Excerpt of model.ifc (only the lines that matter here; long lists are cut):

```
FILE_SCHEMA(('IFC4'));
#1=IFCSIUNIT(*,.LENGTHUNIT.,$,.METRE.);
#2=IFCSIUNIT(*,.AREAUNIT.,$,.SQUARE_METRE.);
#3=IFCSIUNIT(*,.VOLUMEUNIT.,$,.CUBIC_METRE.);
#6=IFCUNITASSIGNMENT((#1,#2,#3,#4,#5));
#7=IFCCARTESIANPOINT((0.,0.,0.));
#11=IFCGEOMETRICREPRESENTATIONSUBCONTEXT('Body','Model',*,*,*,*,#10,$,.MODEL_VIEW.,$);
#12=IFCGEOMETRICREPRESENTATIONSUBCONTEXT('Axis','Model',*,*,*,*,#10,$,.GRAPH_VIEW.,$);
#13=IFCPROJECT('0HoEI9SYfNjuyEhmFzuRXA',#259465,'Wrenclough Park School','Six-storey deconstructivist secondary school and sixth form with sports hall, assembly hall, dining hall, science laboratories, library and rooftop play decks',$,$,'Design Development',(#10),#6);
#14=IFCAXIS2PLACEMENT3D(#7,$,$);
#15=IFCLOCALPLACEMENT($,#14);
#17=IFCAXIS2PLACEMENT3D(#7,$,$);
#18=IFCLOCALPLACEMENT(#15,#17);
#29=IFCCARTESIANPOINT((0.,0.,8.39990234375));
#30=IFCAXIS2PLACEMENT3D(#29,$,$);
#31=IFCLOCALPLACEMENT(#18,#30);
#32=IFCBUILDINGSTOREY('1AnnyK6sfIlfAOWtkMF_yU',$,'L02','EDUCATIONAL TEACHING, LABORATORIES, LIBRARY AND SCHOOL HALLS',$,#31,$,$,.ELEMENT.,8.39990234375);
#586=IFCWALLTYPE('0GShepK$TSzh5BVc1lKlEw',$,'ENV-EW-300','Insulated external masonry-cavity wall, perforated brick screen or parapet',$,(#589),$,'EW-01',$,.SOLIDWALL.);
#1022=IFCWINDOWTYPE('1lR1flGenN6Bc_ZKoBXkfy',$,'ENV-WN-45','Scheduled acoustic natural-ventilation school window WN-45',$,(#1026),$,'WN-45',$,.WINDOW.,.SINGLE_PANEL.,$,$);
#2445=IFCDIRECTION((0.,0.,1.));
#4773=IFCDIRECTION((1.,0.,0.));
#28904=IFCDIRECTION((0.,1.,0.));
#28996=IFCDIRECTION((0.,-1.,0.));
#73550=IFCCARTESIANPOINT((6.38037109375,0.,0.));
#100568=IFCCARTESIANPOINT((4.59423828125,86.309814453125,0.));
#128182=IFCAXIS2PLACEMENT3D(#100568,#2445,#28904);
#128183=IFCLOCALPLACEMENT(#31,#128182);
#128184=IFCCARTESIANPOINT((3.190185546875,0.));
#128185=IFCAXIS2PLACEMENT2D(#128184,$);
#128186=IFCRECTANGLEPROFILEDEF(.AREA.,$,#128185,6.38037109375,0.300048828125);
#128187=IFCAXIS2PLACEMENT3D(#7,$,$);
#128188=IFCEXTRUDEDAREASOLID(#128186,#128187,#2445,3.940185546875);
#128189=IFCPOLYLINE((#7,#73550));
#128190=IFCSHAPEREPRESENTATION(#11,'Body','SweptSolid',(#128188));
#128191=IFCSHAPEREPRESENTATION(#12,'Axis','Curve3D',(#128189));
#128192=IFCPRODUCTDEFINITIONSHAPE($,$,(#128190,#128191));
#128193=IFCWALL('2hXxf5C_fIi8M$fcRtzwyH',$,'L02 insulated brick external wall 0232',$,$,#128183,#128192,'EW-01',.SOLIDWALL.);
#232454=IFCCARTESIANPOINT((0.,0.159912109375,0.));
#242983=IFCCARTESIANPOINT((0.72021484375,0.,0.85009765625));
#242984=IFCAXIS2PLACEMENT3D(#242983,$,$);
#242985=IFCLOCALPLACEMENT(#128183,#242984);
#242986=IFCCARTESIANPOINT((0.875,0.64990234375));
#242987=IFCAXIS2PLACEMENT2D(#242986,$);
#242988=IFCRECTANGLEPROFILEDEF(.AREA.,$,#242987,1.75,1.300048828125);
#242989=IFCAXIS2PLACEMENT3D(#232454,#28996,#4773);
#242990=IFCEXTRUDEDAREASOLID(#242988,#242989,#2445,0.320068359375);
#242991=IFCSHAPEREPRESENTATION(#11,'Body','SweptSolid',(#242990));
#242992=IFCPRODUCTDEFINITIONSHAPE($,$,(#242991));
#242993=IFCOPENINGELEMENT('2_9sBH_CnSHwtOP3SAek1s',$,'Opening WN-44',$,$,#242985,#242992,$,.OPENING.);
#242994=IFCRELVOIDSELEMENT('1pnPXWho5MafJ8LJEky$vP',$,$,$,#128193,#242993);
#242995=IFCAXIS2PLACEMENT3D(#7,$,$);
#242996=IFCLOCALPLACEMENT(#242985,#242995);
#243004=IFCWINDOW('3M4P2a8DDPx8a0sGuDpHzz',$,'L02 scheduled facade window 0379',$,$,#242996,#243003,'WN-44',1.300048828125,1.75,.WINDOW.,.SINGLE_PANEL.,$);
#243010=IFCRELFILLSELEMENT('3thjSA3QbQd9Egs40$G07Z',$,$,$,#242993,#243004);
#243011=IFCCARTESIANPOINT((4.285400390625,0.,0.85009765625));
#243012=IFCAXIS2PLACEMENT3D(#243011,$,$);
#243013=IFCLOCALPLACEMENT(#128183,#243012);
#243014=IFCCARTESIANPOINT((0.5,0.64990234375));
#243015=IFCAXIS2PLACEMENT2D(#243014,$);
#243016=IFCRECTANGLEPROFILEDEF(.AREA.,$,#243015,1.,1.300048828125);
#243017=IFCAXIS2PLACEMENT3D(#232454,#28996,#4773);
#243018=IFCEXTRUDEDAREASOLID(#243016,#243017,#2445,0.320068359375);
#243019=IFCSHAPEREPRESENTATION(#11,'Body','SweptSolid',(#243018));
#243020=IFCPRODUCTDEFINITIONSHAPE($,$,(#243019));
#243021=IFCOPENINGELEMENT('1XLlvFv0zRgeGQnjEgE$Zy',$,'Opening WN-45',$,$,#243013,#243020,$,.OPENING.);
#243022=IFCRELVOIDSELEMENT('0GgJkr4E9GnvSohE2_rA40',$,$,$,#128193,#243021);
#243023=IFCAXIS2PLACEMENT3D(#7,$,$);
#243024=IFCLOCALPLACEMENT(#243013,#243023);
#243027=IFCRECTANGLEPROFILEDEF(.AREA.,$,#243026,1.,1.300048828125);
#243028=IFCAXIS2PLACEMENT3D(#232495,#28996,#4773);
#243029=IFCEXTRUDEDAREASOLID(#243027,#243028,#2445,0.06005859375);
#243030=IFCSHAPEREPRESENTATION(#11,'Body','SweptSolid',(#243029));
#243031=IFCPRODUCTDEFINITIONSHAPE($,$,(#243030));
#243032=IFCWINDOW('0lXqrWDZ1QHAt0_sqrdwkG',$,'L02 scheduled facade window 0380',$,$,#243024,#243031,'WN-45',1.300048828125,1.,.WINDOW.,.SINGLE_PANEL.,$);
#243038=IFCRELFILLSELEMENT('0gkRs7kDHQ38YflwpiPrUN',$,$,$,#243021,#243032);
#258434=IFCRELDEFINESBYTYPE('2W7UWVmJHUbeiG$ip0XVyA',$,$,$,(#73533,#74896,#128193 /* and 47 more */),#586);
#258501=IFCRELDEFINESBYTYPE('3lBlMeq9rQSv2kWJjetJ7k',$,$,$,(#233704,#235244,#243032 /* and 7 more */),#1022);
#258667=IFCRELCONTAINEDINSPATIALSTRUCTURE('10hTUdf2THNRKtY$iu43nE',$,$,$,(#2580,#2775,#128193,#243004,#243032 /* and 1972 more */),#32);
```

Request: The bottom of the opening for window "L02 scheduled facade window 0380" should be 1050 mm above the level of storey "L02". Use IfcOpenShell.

```python
import numpy as np
import ifcopenshell
import ifcopenshell.api.geometry
import ifcopenshell.geom
import ifcopenshell.util.element
import ifcopenshell.util.placement
import ifcopenshell.util.shape
import ifcopenshell.util.unit

model = ifcopenshell.open("model.ifc")
unit_scale = ifcopenshell.util.unit.calculate_unit_scale(model)

window = model.by_id(243032)
opening = window.FillsVoids[0].RelatingOpeningElement
storey = ifcopenshell.util.element.get_container(window, ifc_class="IfcBuildingStorey")
level = ifcopenshell.util.placement.get_local_placement(storey.ObjectPlacement)[2, 3]

# The opening's origin need not be at the sill, so measure its lowest point.
shape = ifcopenshell.geom.create_shape(ifcopenshell.geom.settings(), opening)
bottom = ifcopenshell.util.shape.get_shape_bottom_elevation(shape, shape.geometry) / unit_scale
dz = level + 1.05 / unit_scale - bottom

shift = np.array([0.0, 0.0, dz])
# The window is placed relative to its opening, so it follows when the opening moves.
matrix = ifcopenshell.util.placement.get_local_placement(opening.ObjectPlacement)
matrix[:3, 3] += shift
ifcopenshell.api.geometry.edit_object_placement(
    model, product=opening, matrix=matrix, is_si=False, should_transform_children=True
)

print(f"moved by {dz * unit_scale:+.3f} m")

model.write("model_updated.ifc")
```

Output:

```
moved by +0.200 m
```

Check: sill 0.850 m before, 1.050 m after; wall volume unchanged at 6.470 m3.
